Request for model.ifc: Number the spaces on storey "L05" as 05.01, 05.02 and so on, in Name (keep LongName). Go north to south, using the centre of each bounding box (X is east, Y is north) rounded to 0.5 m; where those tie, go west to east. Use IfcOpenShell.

First a look at what the model holds.

```python
import ifcopenshell
import ifcopenshell.util.element
import ifcopenshell.util.placement

model = ifcopenshell.open("model.ifc")
print(model.schema)
storey = next(s for s in model.by_type("IfcBuildingStorey") if s.Name == "L05")
spaces = [e for e in ifcopenshell.util.element.get_decomposition(storey) if e.is_a("IfcSpace")]
for e in sorted(spaces, key=lambda e: e.id()):
    origin = ifcopenshell.util.placement.get_local_placement(e.ObjectPlacement)[:3, 3]
    print(e.id(), e.Name, e.LongName, origin.round(2) + 0.0, sep=" | ")
```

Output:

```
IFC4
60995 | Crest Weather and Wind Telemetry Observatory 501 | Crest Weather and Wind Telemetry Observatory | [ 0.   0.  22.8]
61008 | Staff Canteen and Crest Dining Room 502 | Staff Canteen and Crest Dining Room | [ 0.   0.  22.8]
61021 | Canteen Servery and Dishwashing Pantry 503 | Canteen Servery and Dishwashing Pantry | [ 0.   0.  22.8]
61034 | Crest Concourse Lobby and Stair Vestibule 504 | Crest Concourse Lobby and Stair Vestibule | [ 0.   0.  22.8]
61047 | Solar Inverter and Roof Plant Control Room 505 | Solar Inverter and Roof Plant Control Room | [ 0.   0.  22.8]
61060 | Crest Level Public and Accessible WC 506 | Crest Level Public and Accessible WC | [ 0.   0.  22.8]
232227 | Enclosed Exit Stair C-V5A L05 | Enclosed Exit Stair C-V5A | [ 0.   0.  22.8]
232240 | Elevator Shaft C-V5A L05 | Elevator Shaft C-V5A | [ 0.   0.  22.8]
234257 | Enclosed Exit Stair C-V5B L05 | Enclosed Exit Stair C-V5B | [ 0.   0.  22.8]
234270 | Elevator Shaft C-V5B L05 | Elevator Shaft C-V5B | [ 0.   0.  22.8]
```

```python
import ifcopenshell
import ifcopenshell.geom
import ifcopenshell.util.element
import ifcopenshell.util.shape

model = ifcopenshell.open("model.ifc")
settings = ifcopenshell.geom.settings()
settings.set("use-world-coords", True)


def centre(element):
    shape = ifcopenshell.geom.create_shape(settings, element)
    return ifcopenshell.util.shape.get_bbox_centroid(shape.geometry)


storey = next(s for s in model.by_type("IfcBuildingStorey") if s.Name == "L05")
spaces = [e for e in ifcopenshell.util.element.get_decomposition(storey) if e.is_a("IfcSpace")]

# Insertion points can sit at a corner or the storey origin, so sort by the geometry (in metres).
centres = {e: centre(e) for e in spaces}
spaces.sort(key=lambda e: (-round(centres[e][1] / 0.5), centres[e][0]))

for i, e in enumerate(spaces, start=1):
    number = f"05.{i:02d}"
    e.Name = number
    print(e.id(), number)

model.write("model_edited.ifc")
```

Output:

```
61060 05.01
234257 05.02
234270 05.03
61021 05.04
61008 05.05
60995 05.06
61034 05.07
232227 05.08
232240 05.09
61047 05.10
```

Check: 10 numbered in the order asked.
